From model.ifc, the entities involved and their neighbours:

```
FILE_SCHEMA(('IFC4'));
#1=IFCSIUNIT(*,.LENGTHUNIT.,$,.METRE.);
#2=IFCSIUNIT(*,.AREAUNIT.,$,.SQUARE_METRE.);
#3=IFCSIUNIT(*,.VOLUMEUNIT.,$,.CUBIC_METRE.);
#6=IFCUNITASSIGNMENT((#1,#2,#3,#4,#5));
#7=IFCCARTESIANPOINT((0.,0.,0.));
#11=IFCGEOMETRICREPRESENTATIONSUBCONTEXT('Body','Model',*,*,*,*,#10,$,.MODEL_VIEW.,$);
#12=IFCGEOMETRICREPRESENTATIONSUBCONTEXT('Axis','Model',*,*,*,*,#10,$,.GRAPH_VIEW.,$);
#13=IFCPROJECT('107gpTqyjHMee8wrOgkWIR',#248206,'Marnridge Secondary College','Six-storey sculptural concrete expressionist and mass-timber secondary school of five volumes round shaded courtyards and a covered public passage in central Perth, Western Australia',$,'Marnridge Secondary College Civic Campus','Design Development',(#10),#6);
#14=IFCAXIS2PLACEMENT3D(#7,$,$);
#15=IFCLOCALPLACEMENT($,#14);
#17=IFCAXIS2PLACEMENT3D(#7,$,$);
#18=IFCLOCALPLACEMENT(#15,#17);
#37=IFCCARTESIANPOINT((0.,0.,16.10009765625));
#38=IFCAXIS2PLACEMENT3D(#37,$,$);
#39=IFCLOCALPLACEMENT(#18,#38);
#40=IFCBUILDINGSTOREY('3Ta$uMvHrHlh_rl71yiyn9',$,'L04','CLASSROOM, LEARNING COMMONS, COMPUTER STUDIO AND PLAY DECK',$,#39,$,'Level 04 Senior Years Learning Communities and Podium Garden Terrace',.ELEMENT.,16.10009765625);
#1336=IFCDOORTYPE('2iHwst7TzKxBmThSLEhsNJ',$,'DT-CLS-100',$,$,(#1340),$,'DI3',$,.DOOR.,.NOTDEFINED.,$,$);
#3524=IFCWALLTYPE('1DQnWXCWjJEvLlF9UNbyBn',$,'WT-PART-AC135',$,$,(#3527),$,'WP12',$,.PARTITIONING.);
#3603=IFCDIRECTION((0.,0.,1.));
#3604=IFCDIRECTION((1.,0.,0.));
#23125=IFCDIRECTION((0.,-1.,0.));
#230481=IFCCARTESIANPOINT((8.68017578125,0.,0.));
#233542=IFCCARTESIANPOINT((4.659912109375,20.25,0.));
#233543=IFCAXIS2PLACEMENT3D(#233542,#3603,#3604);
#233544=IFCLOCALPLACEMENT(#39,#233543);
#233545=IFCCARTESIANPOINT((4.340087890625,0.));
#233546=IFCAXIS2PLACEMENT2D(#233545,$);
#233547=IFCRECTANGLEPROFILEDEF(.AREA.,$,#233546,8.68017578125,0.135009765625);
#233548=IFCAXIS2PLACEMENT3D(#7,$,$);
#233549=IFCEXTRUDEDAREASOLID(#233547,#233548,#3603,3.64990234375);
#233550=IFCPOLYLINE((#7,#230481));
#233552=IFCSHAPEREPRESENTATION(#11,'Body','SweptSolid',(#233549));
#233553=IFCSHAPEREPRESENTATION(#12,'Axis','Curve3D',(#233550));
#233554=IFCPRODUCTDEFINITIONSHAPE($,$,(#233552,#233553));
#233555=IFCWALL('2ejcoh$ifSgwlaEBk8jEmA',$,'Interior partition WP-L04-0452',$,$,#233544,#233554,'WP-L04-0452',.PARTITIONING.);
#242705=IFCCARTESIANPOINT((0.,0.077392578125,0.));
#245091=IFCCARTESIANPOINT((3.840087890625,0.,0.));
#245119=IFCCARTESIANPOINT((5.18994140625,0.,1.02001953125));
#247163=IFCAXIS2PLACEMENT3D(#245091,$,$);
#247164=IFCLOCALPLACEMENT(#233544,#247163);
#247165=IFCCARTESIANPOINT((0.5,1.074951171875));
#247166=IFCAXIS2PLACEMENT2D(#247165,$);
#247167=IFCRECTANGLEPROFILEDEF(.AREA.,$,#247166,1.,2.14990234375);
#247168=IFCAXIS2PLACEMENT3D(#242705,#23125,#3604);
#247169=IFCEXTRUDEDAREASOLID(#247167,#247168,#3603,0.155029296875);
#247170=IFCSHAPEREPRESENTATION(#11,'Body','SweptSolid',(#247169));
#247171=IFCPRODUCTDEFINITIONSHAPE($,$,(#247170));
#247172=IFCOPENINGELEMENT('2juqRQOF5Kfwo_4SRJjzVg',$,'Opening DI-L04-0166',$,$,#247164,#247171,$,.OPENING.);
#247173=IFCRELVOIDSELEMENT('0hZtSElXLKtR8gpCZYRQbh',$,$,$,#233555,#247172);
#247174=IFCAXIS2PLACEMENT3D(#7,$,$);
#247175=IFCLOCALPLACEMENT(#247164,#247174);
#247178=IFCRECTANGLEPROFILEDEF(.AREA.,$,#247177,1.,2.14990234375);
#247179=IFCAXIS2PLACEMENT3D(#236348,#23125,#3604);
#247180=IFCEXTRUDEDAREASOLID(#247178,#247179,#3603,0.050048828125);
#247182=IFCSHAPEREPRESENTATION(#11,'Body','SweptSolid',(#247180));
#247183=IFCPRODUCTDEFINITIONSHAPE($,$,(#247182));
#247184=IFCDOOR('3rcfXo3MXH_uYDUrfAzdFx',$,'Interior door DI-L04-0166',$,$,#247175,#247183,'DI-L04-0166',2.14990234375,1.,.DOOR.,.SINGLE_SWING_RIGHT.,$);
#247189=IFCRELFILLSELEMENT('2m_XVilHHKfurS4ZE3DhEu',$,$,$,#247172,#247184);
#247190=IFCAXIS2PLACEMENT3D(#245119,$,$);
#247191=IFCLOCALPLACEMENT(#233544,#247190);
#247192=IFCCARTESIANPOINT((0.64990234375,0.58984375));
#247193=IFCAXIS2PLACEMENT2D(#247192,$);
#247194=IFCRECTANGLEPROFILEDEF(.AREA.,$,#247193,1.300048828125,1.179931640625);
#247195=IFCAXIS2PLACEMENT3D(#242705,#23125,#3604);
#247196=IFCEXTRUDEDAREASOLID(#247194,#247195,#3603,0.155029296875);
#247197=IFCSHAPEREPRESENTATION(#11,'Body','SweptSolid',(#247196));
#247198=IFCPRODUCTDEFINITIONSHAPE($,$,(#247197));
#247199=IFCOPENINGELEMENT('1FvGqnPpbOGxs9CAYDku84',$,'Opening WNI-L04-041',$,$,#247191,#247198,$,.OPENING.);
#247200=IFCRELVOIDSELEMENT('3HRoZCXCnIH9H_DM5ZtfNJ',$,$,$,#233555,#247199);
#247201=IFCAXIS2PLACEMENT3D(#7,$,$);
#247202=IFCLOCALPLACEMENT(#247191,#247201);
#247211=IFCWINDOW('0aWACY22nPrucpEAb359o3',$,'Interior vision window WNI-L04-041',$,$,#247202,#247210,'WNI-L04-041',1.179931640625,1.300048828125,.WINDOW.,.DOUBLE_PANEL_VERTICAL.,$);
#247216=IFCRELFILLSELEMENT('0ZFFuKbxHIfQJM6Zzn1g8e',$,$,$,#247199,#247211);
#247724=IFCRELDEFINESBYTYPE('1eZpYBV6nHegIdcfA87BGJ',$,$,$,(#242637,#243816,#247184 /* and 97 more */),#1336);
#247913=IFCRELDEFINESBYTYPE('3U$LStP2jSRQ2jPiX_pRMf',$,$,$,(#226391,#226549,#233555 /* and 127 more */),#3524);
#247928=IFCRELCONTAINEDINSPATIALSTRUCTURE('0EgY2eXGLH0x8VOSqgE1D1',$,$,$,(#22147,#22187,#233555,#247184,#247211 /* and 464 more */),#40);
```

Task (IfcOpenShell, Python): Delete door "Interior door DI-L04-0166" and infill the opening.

```python
import ifcopenshell
import ifcopenshell.api.feature
import ifcopenshell.api.root
import ifcopenshell.geom
import ifcopenshell.util.shape

model = ifcopenshell.open("model.ifc")
settings = ifcopenshell.geom.settings()


def volume(element):
    """Net volume in cubic metres, openings subtracted."""
    shape = ifcopenshell.geom.create_shape(settings, element)
    return ifcopenshell.util.shape.get_volume(shape.geometry)


door = model.by_id(247184)
opening = door.FillsVoids[0].RelatingOpeningElement
wall = opening.VoidsElements[0].RelatingBuildingElement
before = volume(wall)

ifcopenshell.api.root.remove_product(model, product=door)
ifcopenshell.api.feature.remove_feature(model, feature=opening)

after = volume(wall)

print(f"wall volume {before:.3f} -> {after:.3f} m3")

model.write("model-out.ifc")
```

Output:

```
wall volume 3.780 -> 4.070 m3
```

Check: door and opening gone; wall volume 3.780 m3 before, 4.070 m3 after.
